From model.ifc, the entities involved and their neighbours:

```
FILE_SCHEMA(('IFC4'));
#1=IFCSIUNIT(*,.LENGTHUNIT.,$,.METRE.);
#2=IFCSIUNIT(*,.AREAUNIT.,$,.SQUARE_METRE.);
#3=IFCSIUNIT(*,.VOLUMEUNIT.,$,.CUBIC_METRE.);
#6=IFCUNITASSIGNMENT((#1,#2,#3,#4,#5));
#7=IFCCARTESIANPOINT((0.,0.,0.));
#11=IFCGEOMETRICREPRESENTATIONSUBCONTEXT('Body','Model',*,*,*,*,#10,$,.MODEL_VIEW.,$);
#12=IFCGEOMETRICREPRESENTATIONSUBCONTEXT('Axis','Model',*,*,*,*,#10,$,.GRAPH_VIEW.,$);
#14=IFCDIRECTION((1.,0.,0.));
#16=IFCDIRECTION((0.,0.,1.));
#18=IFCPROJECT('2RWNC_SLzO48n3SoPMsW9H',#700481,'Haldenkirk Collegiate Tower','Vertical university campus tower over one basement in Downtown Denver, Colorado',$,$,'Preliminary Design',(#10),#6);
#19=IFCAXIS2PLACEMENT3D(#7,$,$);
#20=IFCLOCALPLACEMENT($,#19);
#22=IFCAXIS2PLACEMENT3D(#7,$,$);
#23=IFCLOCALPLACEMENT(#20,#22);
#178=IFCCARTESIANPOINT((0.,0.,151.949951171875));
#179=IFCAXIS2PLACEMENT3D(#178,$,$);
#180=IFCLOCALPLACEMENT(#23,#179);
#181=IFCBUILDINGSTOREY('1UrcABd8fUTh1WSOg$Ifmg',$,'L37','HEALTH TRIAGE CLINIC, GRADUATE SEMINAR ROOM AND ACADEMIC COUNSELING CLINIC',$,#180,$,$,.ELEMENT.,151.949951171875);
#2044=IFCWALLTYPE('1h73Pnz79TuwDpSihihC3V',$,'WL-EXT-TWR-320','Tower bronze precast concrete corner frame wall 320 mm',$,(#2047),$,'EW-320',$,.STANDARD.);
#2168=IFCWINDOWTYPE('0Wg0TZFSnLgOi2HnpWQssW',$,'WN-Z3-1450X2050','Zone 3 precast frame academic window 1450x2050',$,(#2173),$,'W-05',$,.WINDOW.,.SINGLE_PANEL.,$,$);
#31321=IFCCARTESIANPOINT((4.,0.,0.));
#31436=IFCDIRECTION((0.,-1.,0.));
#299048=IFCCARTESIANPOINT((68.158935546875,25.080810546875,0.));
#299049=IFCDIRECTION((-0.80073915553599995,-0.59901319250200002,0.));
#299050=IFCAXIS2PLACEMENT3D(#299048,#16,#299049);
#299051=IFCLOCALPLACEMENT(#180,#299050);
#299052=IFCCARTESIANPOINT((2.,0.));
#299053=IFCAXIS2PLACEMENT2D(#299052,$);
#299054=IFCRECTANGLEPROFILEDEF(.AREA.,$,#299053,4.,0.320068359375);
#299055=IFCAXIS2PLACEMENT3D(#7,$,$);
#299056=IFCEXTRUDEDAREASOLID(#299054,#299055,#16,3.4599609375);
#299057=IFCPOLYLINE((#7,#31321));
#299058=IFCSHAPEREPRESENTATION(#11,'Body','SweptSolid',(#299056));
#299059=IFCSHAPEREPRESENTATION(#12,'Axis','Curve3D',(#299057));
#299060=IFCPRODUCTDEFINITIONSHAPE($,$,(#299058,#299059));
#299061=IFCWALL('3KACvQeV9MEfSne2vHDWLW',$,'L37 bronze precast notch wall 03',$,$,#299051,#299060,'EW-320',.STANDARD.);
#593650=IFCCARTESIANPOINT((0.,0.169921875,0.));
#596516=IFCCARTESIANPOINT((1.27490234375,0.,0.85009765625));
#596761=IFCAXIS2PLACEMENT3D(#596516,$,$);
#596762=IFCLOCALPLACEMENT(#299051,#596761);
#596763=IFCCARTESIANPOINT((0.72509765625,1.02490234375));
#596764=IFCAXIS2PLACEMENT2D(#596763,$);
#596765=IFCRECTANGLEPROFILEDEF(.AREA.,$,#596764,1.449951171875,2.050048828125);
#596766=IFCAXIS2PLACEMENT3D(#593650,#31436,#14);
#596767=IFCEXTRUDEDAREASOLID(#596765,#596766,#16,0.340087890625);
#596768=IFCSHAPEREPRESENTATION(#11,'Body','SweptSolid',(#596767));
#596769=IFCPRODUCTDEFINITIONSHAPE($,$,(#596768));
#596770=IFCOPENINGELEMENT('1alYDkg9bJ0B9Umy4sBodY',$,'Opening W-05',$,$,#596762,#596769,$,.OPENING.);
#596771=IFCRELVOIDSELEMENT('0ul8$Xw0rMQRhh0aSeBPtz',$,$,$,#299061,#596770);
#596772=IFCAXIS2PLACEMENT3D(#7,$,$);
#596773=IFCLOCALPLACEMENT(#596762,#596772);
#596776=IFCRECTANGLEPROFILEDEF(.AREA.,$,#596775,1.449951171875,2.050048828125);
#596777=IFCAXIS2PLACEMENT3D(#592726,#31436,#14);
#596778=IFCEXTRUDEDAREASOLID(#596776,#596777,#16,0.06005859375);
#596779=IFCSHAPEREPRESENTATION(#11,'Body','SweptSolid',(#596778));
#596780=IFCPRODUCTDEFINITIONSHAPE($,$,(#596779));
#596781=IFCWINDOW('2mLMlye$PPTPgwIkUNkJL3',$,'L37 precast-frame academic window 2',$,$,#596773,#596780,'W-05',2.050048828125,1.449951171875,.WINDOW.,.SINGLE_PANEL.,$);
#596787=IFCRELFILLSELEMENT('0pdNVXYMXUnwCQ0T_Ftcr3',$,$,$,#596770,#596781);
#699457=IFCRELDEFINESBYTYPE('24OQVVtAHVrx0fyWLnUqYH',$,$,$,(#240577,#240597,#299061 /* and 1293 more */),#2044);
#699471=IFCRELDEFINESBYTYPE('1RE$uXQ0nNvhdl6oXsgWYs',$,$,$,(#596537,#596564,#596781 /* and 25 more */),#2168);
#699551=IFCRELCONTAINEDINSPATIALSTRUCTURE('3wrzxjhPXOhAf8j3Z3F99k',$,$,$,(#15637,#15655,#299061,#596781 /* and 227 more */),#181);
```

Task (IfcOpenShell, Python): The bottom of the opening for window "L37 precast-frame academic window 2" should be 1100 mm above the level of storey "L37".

```python
import numpy as np
import ifcopenshell
import ifcopenshell.api.geometry
import ifcopenshell.geom
import ifcopenshell.util.element
import ifcopenshell.util.placement
import ifcopenshell.util.shape
import ifcopenshell.util.unit

model = ifcopenshell.open("model.ifc")
unit_scale = ifcopenshell.util.unit.calculate_unit_scale(model)

window = model.by_guid("2mLMlye$PPTPgwIkUNkJL3")
opening = window.FillsVoids[0].RelatingOpeningElement
storey = ifcopenshell.util.element.get_container(window, ifc_class="IfcBuildingStorey")
level = ifcopenshell.util.placement.get_local_placement(storey.ObjectPlacement)[2, 3]

# The opening's origin need not be at the sill, so measure its lowest point.
shape = ifcopenshell.geom.create_shape(ifcopenshell.geom.settings(), opening)
bottom = ifcopenshell.util.shape.get_shape_bottom_elevation(shape, shape.geometry) / unit_scale
dz = level + 1.1 / unit_scale - bottom

shift = np.array([0.0, 0.0, dz])
# The window is placed relative to its opening, so it follows when the opening moves.
matrix = ifcopenshell.util.placement.get_local_placement(opening.ObjectPlacement)
matrix[:3, 3] += shift
ifcopenshell.api.geometry.edit_object_placement(
    model, product=opening, matrix=matrix, is_si=False, should_transform_children=True
)

print(f"moved by {dz * unit_scale:+.3f} m")

model.write("model-out.ifc")
```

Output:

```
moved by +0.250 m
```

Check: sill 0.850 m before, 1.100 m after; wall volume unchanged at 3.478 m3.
